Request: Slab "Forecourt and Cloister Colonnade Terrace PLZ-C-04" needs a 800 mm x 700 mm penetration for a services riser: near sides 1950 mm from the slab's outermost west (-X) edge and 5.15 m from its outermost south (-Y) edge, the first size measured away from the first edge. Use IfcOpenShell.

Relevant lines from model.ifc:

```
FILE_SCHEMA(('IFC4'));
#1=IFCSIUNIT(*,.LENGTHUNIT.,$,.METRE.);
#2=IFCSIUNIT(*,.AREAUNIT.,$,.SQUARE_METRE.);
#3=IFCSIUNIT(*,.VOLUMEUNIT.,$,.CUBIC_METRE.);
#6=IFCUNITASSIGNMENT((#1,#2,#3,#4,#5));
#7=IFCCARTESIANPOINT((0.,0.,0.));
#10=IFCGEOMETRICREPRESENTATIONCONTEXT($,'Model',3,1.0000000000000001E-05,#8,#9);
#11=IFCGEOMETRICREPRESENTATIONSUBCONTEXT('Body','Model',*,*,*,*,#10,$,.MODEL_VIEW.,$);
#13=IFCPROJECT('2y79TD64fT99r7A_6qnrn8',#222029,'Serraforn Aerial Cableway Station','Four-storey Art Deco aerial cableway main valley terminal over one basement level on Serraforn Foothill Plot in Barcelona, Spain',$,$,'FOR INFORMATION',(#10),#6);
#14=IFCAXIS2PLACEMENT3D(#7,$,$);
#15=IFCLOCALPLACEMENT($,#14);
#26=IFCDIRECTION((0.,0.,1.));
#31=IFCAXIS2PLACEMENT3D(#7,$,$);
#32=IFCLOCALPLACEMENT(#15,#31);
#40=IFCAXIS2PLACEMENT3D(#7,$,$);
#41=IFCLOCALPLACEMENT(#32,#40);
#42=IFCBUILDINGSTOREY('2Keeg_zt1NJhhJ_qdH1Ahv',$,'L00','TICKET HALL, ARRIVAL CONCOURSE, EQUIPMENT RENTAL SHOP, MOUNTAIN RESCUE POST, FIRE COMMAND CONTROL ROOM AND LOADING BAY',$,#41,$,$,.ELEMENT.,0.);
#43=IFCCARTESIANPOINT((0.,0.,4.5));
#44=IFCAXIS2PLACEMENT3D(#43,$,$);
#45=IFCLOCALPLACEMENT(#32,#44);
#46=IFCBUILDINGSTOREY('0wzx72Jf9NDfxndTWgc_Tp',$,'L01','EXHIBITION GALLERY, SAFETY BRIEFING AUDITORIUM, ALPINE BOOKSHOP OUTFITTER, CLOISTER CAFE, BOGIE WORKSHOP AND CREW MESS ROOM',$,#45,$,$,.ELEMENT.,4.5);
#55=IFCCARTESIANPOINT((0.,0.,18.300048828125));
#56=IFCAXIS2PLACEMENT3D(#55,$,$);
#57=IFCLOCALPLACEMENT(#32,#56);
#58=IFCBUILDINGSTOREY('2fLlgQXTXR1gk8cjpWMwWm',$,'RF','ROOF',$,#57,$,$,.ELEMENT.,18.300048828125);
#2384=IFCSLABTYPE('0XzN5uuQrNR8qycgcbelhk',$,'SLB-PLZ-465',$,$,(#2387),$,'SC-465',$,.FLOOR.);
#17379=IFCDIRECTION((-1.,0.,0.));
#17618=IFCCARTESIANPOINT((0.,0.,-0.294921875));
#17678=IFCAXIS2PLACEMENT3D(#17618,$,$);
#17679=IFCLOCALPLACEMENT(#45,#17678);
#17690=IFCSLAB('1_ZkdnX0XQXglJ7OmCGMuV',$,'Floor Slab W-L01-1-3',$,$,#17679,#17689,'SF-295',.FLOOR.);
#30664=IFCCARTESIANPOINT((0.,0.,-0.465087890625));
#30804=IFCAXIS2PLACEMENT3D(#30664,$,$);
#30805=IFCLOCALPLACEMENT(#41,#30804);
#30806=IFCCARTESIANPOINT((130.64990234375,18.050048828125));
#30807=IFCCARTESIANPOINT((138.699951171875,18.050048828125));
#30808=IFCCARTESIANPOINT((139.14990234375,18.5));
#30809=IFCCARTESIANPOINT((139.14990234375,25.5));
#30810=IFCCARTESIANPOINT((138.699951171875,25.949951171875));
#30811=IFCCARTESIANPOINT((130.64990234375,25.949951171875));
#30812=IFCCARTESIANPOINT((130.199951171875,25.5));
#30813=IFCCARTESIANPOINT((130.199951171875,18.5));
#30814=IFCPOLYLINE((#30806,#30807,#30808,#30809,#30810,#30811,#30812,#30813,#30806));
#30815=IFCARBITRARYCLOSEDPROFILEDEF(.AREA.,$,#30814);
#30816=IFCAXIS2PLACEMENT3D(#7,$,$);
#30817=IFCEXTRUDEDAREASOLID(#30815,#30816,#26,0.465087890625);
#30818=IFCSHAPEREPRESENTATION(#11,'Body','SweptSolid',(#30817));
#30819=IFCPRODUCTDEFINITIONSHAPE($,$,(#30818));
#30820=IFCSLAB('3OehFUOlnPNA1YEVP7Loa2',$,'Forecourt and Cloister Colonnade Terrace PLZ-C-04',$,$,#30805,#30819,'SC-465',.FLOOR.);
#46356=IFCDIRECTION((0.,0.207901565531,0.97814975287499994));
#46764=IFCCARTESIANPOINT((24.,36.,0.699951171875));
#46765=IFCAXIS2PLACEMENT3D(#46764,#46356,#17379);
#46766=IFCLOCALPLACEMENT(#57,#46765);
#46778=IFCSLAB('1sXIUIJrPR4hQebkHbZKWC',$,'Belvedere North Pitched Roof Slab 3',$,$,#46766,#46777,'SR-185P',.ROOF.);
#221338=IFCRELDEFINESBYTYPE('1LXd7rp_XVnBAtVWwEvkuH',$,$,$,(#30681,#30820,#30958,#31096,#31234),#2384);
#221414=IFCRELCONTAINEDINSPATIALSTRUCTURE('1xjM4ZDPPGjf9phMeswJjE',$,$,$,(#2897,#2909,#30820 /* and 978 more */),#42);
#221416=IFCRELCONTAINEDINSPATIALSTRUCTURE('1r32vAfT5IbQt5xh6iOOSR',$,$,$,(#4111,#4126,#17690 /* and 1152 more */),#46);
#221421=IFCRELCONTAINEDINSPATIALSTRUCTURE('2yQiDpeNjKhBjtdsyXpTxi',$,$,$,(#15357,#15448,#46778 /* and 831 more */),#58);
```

```python
import numpy as np
import ifcopenshell
import ifcopenshell.api.feature
import ifcopenshell.api.geometry
import ifcopenshell.api.root
import ifcopenshell.geom
import ifcopenshell.util.placement
import ifcopenshell.util.representation
import ifcopenshell.util.shape
import ifcopenshell.util.unit

model = ifcopenshell.open("model.ifc")
unit_scale = ifcopenshell.util.unit.calculate_unit_scale(model)
settings = ifcopenshell.geom.settings()


def volume(element):
    """Net volume in cubic metres, openings subtracted."""
    shape = ifcopenshell.geom.create_shape(settings, element)
    return ifcopenshell.util.shape.get_volume(shape.geometry)


slab = model.by_guid("3OehFUOlnPNA1YEVP7Loa2")
before = volume(slab)

# Extent in the slab's own axes, in metres. The edges named are its -X and -Y sides.
slab_shape = ifcopenshell.geom.create_shape(settings, slab)
vertices = ifcopenshell.util.shape.get_vertices(slab_shape.geometry)
x_min, y_min, bottom = vertices.min(axis=0)
top = vertices[:, 2].max()

opening = ifcopenshell.api.root.create_entity(model, ifc_class="IfcOpeningElement", name="Services riser opening", predefined_type="OPENING")
context = ifcopenshell.util.representation.get_context(model, "Model", "Body", "MODEL_VIEW")
width, depth = 0.8, 0.7
outline = [(0.0, 0.0), (width, 0.0), (width, depth), (0.0, depth), (0.0, 0.0)]
# Overshoot both faces by 50 mm so the cut is clean.
shape = ifcopenshell.api.geometry.add_slab_representation(
    model, context=context, depth=top - bottom + 0.1, polyline=outline
)
ifcopenshell.api.geometry.assign_representation(model, product=opening, representation=shape)

matrix = ifcopenshell.util.placement.get_local_placement(slab.ObjectPlacement)
matrix[:, 3] = matrix @ np.append(np.array([x_min + 1.95, y_min + 5.15, bottom - 0.05]) / unit_scale, 1.0)
ifcopenshell.api.geometry.edit_object_placement(model, product=opening, matrix=matrix, is_si=False)
ifcopenshell.api.feature.add_feature(model, feature=opening, element=slab)

after = volume(slab)

print(f"slab volume {before:.3f} -> {after:.3f} m3")

model.write("model_rev.ifc")
```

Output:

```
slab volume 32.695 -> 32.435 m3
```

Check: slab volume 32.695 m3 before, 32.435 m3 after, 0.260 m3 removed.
